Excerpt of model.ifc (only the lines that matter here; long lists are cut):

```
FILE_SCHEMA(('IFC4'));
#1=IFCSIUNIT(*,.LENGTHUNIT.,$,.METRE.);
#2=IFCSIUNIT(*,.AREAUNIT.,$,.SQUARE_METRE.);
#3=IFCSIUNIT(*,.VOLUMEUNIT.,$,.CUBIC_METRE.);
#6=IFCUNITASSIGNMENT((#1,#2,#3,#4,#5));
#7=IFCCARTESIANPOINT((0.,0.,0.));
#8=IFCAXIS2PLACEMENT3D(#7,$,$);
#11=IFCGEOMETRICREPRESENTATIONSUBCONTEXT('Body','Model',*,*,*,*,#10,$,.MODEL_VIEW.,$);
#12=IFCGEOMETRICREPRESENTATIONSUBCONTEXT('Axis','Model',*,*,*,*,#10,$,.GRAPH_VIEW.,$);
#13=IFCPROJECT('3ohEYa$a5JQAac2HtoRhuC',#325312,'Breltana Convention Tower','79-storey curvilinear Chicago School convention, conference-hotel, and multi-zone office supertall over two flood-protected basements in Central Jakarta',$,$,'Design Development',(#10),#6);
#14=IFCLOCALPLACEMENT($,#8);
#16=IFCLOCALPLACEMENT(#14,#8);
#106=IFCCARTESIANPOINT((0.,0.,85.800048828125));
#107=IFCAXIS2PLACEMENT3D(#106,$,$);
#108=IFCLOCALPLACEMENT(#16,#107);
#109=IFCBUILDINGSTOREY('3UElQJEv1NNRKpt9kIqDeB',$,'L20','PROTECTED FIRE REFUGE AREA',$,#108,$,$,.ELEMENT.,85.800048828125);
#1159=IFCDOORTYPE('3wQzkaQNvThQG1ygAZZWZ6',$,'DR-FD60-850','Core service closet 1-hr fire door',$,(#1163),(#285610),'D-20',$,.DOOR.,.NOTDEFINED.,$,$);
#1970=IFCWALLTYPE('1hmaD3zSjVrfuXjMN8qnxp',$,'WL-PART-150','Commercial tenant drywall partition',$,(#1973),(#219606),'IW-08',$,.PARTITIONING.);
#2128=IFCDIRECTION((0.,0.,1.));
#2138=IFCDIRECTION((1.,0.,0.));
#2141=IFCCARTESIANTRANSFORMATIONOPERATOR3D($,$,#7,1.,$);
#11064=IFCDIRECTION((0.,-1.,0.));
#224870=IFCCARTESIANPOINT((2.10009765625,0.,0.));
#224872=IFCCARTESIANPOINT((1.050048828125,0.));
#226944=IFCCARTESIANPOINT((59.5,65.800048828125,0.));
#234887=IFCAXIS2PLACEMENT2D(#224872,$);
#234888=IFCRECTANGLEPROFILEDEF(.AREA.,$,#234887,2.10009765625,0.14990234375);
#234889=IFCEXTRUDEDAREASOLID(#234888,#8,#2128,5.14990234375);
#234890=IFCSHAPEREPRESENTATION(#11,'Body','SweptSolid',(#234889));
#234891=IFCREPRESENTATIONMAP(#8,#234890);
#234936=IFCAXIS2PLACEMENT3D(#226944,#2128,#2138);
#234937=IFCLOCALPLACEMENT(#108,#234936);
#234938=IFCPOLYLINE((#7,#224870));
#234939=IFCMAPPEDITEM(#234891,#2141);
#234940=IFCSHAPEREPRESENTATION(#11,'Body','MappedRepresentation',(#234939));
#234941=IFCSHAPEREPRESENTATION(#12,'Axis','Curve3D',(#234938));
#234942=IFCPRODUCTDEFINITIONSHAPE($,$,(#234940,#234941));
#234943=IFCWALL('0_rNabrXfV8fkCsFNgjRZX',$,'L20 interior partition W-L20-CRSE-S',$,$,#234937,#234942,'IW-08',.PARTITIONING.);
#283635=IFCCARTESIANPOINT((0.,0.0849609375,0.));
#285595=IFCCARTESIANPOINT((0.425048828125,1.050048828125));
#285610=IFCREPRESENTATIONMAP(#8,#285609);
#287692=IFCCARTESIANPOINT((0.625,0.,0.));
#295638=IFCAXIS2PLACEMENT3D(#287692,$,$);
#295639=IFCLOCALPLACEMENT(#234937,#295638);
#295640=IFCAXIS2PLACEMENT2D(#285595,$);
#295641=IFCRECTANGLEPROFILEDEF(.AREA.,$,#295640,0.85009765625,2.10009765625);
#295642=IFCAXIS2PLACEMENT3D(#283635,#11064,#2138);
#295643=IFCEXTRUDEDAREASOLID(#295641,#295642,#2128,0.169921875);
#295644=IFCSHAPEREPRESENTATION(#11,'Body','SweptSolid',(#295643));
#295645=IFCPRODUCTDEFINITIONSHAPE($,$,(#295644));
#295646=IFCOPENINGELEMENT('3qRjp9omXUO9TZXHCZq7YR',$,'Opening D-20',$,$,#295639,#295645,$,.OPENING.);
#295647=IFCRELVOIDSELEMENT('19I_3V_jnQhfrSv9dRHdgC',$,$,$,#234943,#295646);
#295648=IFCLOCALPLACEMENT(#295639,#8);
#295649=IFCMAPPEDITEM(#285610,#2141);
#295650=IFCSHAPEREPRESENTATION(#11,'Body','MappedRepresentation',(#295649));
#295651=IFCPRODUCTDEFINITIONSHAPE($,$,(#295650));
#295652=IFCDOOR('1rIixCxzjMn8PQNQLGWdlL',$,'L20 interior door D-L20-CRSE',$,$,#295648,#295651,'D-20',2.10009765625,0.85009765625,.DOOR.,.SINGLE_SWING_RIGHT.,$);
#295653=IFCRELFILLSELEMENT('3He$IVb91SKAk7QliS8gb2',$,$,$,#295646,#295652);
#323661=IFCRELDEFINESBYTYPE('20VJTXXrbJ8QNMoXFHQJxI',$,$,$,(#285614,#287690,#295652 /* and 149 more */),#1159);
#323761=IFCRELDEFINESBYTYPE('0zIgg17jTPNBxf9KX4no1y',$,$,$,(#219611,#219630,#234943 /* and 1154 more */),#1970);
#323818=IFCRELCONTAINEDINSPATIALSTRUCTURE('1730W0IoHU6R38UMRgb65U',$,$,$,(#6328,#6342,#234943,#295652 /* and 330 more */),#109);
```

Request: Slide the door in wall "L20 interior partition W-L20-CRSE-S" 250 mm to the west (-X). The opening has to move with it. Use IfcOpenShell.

```python
import ifcopenshell
import ifcopenshell.api.geometry
import ifcopenshell.util.placement

model = ifcopenshell.open("model.ifc")

door = model.by_guid("1rIixCxzjMn8PQNQLGWdlL")
opening = door.FillsVoids[0].RelatingOpeningElement
wall = opening.VoidsElements[0].RelatingBuildingElement

wall_matrix = ifcopenshell.util.placement.get_local_placement(wall.ObjectPlacement)
shift = wall_matrix[:3, 0] * -0.25
before = ifcopenshell.util.placement.get_local_placement(door.ObjectPlacement)[:3, 3].copy()

# The door is placed relative to its opening, so it follows when the opening moves.
matrix = ifcopenshell.util.placement.get_local_placement(opening.ObjectPlacement)
matrix[:3, 3] += shift
ifcopenshell.api.geometry.edit_object_placement(
    model, product=opening, matrix=matrix, is_si=False, should_transform_children=True
)

after = ifcopenshell.util.placement.get_local_placement(door.ObjectPlacement)[:3, 3]
print("door moved by", (after - before).round(3) + 0.0)

model.write("model-out.ifc")
```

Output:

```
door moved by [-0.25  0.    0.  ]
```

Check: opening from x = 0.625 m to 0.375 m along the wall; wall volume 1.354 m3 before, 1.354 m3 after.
